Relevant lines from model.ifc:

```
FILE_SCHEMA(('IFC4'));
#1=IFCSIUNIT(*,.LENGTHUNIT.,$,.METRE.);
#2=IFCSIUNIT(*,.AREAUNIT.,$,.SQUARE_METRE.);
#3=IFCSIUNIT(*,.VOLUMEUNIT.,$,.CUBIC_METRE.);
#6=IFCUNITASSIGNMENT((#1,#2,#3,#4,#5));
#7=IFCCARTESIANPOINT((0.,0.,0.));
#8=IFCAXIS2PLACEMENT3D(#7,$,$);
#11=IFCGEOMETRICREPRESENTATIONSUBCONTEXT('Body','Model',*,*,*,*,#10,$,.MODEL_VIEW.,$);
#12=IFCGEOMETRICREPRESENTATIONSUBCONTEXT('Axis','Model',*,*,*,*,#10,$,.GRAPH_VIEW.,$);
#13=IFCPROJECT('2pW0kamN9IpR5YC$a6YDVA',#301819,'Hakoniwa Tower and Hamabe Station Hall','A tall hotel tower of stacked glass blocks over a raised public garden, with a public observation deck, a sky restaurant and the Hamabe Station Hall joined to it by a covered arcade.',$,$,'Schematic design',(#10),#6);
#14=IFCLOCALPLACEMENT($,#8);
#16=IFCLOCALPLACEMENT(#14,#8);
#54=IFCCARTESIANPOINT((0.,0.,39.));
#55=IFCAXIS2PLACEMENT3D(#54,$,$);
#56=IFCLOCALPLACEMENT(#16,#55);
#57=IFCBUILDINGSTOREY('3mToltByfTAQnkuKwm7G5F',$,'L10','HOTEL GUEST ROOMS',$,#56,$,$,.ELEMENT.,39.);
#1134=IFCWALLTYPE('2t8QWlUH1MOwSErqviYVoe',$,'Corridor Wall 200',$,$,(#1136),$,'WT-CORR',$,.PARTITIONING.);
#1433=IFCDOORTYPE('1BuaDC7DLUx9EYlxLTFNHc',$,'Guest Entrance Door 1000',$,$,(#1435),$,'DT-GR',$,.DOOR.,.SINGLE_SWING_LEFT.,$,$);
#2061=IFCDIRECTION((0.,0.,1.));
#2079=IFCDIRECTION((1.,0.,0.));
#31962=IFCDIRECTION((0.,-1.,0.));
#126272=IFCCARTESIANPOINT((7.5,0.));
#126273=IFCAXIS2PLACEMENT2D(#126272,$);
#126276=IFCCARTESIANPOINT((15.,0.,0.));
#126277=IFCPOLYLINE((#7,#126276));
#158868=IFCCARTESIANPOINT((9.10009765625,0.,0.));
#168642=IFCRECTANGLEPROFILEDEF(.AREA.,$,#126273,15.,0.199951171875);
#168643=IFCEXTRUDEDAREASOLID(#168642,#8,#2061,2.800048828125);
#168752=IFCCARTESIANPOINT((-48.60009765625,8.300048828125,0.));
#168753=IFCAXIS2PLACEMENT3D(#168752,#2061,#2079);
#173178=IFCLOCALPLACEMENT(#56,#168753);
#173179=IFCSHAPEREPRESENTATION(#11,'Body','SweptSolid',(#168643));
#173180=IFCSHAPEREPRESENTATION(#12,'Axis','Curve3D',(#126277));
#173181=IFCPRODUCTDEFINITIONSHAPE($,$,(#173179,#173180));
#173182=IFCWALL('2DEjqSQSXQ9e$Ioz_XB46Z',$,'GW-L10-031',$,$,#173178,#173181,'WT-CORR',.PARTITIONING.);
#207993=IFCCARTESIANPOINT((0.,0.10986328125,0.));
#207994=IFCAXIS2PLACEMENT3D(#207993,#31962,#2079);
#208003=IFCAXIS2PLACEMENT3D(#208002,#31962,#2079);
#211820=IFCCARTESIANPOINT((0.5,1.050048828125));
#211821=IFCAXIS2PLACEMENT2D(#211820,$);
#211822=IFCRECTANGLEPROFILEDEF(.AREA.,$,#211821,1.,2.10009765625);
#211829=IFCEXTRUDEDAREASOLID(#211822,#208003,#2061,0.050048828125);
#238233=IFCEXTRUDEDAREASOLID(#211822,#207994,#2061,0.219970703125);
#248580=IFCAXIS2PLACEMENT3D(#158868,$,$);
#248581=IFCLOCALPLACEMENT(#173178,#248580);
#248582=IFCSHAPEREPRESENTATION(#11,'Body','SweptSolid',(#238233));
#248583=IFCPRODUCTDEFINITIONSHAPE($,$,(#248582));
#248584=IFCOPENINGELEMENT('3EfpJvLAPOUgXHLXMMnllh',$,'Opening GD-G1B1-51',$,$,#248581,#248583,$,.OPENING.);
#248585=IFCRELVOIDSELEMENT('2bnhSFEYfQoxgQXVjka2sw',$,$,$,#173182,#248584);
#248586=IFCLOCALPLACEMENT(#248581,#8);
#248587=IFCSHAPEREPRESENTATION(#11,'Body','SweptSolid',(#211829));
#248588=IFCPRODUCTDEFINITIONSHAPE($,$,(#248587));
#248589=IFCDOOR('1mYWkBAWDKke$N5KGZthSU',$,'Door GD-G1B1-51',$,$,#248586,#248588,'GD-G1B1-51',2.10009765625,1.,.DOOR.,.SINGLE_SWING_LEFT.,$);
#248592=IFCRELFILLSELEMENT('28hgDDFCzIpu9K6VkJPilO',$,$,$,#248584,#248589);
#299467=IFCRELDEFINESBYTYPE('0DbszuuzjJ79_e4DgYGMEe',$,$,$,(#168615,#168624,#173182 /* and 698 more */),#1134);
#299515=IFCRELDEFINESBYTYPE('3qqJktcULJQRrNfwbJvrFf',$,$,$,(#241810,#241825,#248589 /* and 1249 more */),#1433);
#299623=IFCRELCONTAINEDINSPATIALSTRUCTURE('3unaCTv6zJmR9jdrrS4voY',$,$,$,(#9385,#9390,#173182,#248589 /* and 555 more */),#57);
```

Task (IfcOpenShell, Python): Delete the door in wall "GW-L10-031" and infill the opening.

```python
import ifcopenshell
import ifcopenshell.api.feature
import ifcopenshell.api.root
import ifcopenshell.geom
import ifcopenshell.util.shape

model = ifcopenshell.open("model.ifc")
settings = ifcopenshell.geom.settings()


def volume(element):
    """Net volume in cubic metres, openings subtracted."""
    shape = ifcopenshell.geom.create_shape(settings, element)
    return ifcopenshell.util.shape.get_volume(shape.geometry)


door = model.by_id(248589)
opening = door.FillsVoids[0].RelatingOpeningElement
wall = opening.VoidsElements[0].RelatingBuildingElement
before = volume(wall)

ifcopenshell.api.root.remove_product(model, product=door)
ifcopenshell.api.feature.remove_feature(model, feature=opening)

after = volume(wall)

print(f"wall volume {before:.3f} -> {after:.3f} m3")

model.write("model_updated.ifc")
```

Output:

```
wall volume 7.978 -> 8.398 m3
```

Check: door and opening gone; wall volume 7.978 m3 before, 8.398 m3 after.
